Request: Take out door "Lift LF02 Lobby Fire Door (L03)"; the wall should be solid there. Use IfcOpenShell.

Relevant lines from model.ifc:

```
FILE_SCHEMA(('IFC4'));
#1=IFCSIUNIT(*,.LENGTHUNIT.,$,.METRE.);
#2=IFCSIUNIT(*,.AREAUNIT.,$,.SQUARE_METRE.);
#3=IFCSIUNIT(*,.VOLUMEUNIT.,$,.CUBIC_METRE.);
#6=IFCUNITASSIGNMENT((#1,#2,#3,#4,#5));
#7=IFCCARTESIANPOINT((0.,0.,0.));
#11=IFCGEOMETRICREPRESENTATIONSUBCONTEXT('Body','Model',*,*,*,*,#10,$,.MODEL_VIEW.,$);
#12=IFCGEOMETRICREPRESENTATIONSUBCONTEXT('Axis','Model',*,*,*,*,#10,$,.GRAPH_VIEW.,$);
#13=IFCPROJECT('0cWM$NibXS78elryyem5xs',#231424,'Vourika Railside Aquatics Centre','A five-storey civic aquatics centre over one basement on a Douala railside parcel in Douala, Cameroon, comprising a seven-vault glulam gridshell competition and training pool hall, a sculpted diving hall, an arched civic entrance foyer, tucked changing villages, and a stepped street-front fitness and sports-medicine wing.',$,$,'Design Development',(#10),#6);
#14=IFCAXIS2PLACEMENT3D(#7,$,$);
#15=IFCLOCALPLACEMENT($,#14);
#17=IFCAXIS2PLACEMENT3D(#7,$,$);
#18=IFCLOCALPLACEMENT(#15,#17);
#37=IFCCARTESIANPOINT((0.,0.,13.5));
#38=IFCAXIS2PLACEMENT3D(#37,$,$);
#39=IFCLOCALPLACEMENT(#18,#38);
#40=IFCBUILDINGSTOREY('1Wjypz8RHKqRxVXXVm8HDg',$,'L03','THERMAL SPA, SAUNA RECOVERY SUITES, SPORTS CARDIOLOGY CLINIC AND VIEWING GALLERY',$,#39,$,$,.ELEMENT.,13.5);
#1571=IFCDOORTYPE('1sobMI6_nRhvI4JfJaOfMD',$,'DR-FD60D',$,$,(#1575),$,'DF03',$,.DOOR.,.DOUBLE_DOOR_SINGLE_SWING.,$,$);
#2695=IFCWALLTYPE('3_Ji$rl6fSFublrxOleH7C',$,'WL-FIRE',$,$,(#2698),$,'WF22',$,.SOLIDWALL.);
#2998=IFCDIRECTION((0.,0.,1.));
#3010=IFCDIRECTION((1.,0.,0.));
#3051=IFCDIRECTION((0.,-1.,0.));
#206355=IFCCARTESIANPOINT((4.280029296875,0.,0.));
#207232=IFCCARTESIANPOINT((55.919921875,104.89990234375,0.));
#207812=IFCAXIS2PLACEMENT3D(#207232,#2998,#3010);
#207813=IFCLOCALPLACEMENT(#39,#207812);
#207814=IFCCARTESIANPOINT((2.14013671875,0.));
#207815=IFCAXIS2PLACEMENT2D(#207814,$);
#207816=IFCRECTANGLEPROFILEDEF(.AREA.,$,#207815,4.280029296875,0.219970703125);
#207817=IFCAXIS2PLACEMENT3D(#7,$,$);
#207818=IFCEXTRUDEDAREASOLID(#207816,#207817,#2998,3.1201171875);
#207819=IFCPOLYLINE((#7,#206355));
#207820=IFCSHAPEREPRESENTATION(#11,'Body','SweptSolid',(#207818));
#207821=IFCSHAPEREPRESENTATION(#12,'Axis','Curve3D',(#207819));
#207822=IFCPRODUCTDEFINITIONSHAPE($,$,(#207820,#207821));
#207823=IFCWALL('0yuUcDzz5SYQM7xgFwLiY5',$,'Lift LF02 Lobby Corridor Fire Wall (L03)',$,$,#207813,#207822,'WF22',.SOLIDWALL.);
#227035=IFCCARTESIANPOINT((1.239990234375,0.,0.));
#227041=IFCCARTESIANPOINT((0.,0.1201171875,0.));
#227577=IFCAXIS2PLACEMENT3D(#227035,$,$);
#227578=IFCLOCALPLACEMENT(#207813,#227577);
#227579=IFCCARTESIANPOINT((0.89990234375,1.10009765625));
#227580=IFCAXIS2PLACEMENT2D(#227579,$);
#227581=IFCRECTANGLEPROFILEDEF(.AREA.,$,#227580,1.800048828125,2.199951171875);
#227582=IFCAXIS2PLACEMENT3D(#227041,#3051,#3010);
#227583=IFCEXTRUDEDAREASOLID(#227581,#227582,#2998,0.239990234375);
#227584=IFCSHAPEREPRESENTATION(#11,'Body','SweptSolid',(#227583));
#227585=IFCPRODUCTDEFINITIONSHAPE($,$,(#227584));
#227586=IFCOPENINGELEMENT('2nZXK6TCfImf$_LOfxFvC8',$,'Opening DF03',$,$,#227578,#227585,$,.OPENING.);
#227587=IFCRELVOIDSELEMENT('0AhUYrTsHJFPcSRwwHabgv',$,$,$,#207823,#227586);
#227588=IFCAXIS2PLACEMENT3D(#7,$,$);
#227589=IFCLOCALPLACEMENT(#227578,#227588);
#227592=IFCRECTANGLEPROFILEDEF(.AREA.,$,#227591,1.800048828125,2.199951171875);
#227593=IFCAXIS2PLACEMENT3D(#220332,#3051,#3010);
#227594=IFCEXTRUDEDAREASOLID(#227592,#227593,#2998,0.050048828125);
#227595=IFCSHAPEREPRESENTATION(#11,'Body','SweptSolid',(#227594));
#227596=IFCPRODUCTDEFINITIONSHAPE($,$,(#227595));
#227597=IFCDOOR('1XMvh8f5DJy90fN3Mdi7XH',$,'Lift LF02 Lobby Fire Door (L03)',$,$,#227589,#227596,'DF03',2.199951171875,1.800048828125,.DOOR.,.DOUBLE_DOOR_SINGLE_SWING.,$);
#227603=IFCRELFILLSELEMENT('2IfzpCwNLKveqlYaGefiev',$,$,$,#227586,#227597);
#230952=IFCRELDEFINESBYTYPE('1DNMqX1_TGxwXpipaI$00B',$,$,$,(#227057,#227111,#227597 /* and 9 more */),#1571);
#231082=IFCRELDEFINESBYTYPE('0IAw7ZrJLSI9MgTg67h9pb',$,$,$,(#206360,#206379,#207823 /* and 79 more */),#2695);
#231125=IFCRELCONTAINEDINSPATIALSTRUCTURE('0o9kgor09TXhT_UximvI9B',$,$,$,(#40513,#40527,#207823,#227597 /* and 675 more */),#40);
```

```python
import ifcopenshell
import ifcopenshell.api.feature
import ifcopenshell.api.root
import ifcopenshell.geom
import ifcopenshell.util.shape

model = ifcopenshell.open("model.ifc")
settings = ifcopenshell.geom.settings()


def volume(element):
    """Net volume in cubic metres, openings subtracted."""
    shape = ifcopenshell.geom.create_shape(settings, element)
    return ifcopenshell.util.shape.get_volume(shape.geometry)


door = model.by_id(227597)
opening = door.FillsVoids[0].RelatingOpeningElement
wall = opening.VoidsElements[0].RelatingBuildingElement
before = volume(wall)

ifcopenshell.api.root.remove_product(model, product=door)
ifcopenshell.api.feature.remove_feature(model, feature=opening)

after = volume(wall)

print(f"wall volume {before:.3f} -> {after:.3f} m3")

model.write("model_updated.ifc")
```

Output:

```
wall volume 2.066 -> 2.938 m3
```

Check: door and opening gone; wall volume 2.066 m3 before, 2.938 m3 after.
